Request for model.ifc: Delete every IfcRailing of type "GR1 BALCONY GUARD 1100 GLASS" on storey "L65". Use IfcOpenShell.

First a look at what the model holds.

```python
import ifcopenshell
import ifcopenshell.util.element

model = ifcopenshell.open("model.ifc")
print(model.schema)
storey = next(s for s in model.by_type("IfcBuildingStorey") if s.Name == "L65")
railings = [e for e in ifcopenshell.util.element.get_decomposition(storey) if e.is_a("IfcRailing")]
seen = {}
for e in railings:
    element_type = ifcopenshell.util.element.get_type(e)
    name = element_type.Name if element_type not in (None, e) else None
    seen[name] = seen.get(name, 0) + 1
for name, count in sorted(seen.items(), key=str):
    print(count, "x", name)
```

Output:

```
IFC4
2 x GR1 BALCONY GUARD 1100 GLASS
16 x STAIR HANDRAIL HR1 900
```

```python
import ifcopenshell
import ifcopenshell.api.root
import ifcopenshell.util.element

model = ifcopenshell.open("model.ifc")

storey = next(s for s in model.by_type("IfcBuildingStorey") if s.Name == "L65")
railings = [e for e in ifcopenshell.util.element.get_decomposition(storey) if e.is_a("IfcRailing")]
targets = [e for e in railings if (t := ifcopenshell.util.element.get_type(e)) not in (None, e) and t.Name == "GR1 BALCONY GUARD 1100 GLASS"]

for e in targets:
    ifcopenshell.api.root.remove_product(model, product=e)
print(len(targets), "removed")

model.write("model_v2.ifc")
```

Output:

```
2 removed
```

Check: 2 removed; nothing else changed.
